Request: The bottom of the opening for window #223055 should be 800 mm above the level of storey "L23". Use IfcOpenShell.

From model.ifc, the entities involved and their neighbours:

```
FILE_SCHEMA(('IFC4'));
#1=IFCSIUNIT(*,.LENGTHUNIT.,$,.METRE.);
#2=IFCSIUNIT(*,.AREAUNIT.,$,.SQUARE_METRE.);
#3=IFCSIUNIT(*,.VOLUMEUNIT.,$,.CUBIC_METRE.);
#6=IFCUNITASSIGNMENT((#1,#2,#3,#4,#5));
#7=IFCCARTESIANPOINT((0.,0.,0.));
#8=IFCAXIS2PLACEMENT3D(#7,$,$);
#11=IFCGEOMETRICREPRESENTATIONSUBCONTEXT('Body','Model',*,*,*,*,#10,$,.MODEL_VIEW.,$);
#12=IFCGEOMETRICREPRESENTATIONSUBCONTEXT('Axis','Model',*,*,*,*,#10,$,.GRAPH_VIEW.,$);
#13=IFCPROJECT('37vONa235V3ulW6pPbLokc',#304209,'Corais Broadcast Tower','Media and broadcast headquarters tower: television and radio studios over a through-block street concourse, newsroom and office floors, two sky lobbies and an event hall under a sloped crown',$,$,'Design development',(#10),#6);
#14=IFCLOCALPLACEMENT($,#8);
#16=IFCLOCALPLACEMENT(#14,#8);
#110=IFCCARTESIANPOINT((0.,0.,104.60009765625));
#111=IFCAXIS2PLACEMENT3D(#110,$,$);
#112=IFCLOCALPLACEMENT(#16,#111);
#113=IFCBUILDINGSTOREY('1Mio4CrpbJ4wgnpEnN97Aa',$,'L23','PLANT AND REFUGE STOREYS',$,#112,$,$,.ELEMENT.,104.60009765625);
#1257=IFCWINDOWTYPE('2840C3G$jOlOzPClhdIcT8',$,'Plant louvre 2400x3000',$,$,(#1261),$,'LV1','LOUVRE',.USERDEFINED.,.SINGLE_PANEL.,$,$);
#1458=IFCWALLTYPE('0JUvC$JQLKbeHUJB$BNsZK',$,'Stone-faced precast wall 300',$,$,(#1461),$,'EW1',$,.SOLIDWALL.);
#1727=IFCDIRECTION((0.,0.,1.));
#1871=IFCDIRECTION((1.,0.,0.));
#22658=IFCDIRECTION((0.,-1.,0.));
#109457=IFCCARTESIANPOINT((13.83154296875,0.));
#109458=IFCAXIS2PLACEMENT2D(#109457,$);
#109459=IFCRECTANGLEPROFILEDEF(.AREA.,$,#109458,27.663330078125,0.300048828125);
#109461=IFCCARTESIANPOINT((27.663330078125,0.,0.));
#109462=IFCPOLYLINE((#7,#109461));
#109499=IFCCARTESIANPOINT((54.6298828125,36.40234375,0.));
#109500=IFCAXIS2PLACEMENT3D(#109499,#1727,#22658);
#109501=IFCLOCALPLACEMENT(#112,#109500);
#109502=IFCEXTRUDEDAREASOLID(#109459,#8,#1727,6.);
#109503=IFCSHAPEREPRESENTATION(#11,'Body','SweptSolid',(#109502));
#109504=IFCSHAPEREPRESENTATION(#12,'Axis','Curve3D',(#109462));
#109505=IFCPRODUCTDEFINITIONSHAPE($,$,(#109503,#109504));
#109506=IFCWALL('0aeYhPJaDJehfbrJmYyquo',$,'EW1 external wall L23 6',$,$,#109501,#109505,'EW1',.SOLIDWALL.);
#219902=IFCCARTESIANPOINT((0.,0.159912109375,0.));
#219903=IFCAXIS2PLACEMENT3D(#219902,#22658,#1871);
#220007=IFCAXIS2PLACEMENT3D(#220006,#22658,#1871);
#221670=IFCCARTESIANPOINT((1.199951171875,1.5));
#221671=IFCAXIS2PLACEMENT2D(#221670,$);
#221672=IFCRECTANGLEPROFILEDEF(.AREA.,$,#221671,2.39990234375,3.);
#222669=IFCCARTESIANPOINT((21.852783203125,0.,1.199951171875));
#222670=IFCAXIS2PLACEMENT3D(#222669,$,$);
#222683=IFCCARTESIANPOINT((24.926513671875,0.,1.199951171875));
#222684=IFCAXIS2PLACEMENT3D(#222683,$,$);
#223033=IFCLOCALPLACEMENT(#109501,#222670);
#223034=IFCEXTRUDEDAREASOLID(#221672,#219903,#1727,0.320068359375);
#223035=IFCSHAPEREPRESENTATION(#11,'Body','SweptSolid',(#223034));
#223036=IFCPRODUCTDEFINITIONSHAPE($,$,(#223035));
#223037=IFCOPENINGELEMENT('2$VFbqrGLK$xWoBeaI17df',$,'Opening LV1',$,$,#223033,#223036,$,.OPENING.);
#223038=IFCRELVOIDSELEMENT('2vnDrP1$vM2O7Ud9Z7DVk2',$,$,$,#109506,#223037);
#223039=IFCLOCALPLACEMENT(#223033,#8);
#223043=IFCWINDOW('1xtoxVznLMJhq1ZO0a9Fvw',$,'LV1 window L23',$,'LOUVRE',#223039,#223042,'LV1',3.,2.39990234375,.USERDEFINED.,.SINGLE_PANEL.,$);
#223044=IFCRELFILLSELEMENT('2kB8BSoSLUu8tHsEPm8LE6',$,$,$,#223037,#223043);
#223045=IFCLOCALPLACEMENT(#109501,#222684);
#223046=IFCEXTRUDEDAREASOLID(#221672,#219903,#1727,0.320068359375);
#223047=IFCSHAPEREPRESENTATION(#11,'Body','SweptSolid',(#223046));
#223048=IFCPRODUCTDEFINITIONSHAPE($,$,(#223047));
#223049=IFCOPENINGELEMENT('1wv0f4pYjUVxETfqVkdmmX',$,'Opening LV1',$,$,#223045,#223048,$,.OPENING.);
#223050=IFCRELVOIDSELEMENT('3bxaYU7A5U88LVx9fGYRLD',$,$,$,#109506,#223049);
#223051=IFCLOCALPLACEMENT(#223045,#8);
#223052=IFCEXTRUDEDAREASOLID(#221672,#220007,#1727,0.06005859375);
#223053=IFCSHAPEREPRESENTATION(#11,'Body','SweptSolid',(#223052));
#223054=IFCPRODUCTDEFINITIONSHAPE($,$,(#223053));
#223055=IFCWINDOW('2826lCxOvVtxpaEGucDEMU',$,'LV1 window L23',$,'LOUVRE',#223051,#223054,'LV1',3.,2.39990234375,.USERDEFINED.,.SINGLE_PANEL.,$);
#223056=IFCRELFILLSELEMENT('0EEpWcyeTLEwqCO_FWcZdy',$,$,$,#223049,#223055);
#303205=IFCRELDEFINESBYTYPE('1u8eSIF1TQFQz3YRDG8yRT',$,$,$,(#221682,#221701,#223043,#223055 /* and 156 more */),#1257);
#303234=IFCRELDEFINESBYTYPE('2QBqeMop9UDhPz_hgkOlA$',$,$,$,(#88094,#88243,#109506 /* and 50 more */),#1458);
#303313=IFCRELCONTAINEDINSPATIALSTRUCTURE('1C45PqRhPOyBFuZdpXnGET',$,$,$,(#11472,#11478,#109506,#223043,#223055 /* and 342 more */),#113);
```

```python
import numpy as np
import ifcopenshell
import ifcopenshell.api.geometry
import ifcopenshell.geom
import ifcopenshell.util.element
import ifcopenshell.util.placement
import ifcopenshell.util.shape
import ifcopenshell.util.unit

model = ifcopenshell.open("model.ifc")
unit_scale = ifcopenshell.util.unit.calculate_unit_scale(model)

window = model.by_id(223055)
opening = window.FillsVoids[0].RelatingOpeningElement
storey = ifcopenshell.util.element.get_container(window, ifc_class="IfcBuildingStorey")
level = ifcopenshell.util.placement.get_local_placement(storey.ObjectPlacement)[2, 3]

# The opening's origin need not be at the sill, so measure its lowest point.
shape = ifcopenshell.geom.create_shape(ifcopenshell.geom.settings(), opening)
bottom = ifcopenshell.util.shape.get_shape_bottom_elevation(shape, shape.geometry) / unit_scale
dz = level + 0.8 - bottom

shift = np.array([0.0, 0.0, dz])
# The window is placed relative to its opening, so it follows when the opening moves.
matrix = ifcopenshell.util.placement.get_local_placement(opening.ObjectPlacement)
matrix[:3, 3] += shift
ifcopenshell.api.geometry.edit_object_placement(
    model, product=opening, matrix=matrix, is_si=False, should_transform_children=True
)

print(f"moved by {dz * unit_scale:+.3f} m")

model.write("model_v2.ifc")
```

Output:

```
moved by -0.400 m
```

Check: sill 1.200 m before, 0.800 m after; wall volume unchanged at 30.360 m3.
